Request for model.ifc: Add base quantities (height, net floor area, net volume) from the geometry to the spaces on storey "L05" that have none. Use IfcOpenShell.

First a look at what the model holds.

```python
import ifcopenshell
import ifcopenshell.util.element
import ifcopenshell.util.unit

model = ifcopenshell.open("model.ifc")
print(model.schema)
for unit_type in ("LENGTHUNIT", "AREAUNIT", "VOLUMEUNIT"):
    print(unit_type, ifcopenshell.util.unit.calculate_unit_scale(model, unit_type))
storey = next(s for s in model.by_type("IfcBuildingStorey") if s.Name == "L05")
spaces = [e for e in ifcopenshell.util.element.get_decomposition(storey) if e.is_a("IfcSpace")]
for e in sorted(spaces, key=lambda e: e.id()):
    print(e.id(), e.is_a(), e.Name, list(ifcopenshell.util.element.get_psets(e, qtos_only=True)), sep=" | ")
```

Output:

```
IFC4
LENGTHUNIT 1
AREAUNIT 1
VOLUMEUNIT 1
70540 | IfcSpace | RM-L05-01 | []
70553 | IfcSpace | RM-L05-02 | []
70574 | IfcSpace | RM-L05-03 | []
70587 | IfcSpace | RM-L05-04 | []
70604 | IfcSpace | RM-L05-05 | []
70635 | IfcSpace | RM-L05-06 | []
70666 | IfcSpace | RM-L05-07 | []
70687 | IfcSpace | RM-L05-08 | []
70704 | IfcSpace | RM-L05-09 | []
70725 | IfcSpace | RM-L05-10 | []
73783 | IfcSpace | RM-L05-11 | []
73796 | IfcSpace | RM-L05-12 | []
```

```python
import ifcopenshell
import ifcopenshell.api.pset
import ifcopenshell.geom
import ifcopenshell.util.element
import ifcopenshell.util.shape
import ifcopenshell.util.unit

model = ifcopenshell.open("model.ifc")
unit_scale = ifcopenshell.util.unit.calculate_unit_scale(model)
area_scale = ifcopenshell.util.unit.calculate_unit_scale(model, "AREAUNIT")
volume_scale = ifcopenshell.util.unit.calculate_unit_scale(model, "VOLUMEUNIT")
settings = ifcopenshell.geom.settings()

storey = next(s for s in model.by_type("IfcBuildingStorey") if s.Name == "L05")
spaces = [e for e in ifcopenshell.util.element.get_decomposition(storey) if e.is_a("IfcSpace")]

for e in sorted(spaces, key=lambda e: e.id()):
    if ifcopenshell.util.element.get_psets(e, qtos_only=True, should_inherit=False):
        continue
    # Geometry comes back in metres, in the element's own axes.
    shape = ifcopenshell.geom.create_shape(settings, e)
    values = {
        "Height": ifcopenshell.util.shape.get_z(shape.geometry) / unit_scale,
        "NetFloorArea": ifcopenshell.util.shape.get_footprint_area(shape.geometry) / area_scale,
        "NetVolume": ifcopenshell.util.shape.get_volume(shape.geometry) / volume_scale,
    }
    qto = ifcopenshell.api.pset.add_qto(model, product=e, name="Qto_SpaceBaseQuantities")
    ifcopenshell.api.pset.edit_qto(model, qto=qto, properties=values)
    print(e.id(), {k: round(v, 3) for k, v in values.items()})

model.write("model_v2.ifc")
```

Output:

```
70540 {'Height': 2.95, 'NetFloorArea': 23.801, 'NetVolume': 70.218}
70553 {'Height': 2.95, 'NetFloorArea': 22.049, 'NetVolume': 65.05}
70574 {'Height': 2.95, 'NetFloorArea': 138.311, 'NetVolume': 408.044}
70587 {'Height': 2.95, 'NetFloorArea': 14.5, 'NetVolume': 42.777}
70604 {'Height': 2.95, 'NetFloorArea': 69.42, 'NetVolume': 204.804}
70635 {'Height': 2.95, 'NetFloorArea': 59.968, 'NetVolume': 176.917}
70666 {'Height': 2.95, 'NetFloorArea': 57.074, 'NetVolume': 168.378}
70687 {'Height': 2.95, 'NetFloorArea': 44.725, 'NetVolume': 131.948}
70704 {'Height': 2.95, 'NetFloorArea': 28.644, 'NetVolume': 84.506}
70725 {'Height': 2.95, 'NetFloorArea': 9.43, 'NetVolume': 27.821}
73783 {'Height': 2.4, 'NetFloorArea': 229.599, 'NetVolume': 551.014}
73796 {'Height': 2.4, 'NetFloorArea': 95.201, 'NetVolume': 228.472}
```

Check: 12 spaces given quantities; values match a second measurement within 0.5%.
